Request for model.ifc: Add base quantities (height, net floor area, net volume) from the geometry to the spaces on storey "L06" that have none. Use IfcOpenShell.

First a look at what the model holds.

```python
import ifcopenshell
import ifcopenshell.util.element
import ifcopenshell.util.unit

model = ifcopenshell.open("model.ifc")
print(model.schema)
for unit_type in ("LENGTHUNIT", "AREAUNIT", "VOLUMEUNIT"):
    print(unit_type, ifcopenshell.util.unit.calculate_unit_scale(model, unit_type))
storey = next(s for s in model.by_type("IfcBuildingStorey") if s.Name == "L06")
spaces = [e for e in ifcopenshell.util.element.get_decomposition(storey) if e.is_a("IfcSpace")]
for e in sorted(spaces, key=lambda e: e.id()):
    print(e.id(), e.is_a(), e.Name, list(ifcopenshell.util.element.get_psets(e, qtos_only=True)), sep=" | ")
```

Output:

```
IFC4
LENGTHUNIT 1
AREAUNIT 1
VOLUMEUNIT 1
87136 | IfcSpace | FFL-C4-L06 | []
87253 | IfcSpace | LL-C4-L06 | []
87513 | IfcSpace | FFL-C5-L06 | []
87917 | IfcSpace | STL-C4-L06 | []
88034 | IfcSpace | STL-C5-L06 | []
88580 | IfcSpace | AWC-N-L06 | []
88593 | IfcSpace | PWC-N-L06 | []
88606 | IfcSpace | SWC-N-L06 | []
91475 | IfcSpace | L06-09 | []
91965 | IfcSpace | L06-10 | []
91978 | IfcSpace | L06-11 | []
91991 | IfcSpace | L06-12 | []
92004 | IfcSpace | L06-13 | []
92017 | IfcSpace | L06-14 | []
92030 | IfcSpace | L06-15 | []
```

```python
import ifcopenshell
import ifcopenshell.api.pset
import ifcopenshell.geom
import ifcopenshell.util.element
import ifcopenshell.util.shape
import ifcopenshell.util.unit

model = ifcopenshell.open("model.ifc")
unit_scale = ifcopenshell.util.unit.calculate_unit_scale(model)
area_scale = ifcopenshell.util.unit.calculate_unit_scale(model, "AREAUNIT")
volume_scale = ifcopenshell.util.unit.calculate_unit_scale(model, "VOLUMEUNIT")
settings = ifcopenshell.geom.settings()

storey = next(s for s in model.by_type("IfcBuildingStorey") if s.Name == "L06")
spaces = [e for e in ifcopenshell.util.element.get_decomposition(storey) if e.is_a("IfcSpace")]

for e in sorted(spaces, key=lambda e: e.id()):
    if ifcopenshell.util.element.get_psets(e, qtos_only=True, should_inherit=False):
        continue
    # Geometry comes back in metres, in the element's own axes.
    shape = ifcopenshell.geom.create_shape(settings, e)
    values = {
        "Height": ifcopenshell.util.shape.get_z(shape.geometry) / unit_scale,
        "NetFloorArea": ifcopenshell.util.shape.get_footprint_area(shape.geometry) / area_scale,
        "NetVolume": ifcopenshell.util.shape.get_volume(shape.geometry) / volume_scale,
    }
    qto = ifcopenshell.api.pset.add_qto(model, product=e, name="Qto_SpaceBaseQuantities")
    ifcopenshell.api.pset.edit_qto(model, qto=qto, properties=values)
    print(e.id(), {k: round(v, 3) for k, v in values.items()})

model.write("model-out.ifc")
```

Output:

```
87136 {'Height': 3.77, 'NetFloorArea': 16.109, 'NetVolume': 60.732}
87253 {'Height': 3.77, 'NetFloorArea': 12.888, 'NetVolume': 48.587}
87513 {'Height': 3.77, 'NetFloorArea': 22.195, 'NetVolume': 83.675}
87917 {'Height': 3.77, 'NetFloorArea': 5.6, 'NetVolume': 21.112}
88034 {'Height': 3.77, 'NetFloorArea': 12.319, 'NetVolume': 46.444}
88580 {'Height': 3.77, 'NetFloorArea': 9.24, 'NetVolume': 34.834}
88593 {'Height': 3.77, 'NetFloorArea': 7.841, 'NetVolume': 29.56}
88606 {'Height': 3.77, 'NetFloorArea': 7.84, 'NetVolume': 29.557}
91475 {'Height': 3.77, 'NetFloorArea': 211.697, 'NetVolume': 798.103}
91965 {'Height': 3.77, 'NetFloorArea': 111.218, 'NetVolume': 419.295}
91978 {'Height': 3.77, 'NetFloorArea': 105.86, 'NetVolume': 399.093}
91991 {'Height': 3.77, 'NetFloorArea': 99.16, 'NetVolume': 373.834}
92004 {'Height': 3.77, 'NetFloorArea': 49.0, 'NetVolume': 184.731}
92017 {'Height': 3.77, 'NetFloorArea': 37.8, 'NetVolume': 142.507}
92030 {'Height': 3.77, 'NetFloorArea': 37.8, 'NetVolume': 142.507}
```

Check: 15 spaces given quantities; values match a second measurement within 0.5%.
